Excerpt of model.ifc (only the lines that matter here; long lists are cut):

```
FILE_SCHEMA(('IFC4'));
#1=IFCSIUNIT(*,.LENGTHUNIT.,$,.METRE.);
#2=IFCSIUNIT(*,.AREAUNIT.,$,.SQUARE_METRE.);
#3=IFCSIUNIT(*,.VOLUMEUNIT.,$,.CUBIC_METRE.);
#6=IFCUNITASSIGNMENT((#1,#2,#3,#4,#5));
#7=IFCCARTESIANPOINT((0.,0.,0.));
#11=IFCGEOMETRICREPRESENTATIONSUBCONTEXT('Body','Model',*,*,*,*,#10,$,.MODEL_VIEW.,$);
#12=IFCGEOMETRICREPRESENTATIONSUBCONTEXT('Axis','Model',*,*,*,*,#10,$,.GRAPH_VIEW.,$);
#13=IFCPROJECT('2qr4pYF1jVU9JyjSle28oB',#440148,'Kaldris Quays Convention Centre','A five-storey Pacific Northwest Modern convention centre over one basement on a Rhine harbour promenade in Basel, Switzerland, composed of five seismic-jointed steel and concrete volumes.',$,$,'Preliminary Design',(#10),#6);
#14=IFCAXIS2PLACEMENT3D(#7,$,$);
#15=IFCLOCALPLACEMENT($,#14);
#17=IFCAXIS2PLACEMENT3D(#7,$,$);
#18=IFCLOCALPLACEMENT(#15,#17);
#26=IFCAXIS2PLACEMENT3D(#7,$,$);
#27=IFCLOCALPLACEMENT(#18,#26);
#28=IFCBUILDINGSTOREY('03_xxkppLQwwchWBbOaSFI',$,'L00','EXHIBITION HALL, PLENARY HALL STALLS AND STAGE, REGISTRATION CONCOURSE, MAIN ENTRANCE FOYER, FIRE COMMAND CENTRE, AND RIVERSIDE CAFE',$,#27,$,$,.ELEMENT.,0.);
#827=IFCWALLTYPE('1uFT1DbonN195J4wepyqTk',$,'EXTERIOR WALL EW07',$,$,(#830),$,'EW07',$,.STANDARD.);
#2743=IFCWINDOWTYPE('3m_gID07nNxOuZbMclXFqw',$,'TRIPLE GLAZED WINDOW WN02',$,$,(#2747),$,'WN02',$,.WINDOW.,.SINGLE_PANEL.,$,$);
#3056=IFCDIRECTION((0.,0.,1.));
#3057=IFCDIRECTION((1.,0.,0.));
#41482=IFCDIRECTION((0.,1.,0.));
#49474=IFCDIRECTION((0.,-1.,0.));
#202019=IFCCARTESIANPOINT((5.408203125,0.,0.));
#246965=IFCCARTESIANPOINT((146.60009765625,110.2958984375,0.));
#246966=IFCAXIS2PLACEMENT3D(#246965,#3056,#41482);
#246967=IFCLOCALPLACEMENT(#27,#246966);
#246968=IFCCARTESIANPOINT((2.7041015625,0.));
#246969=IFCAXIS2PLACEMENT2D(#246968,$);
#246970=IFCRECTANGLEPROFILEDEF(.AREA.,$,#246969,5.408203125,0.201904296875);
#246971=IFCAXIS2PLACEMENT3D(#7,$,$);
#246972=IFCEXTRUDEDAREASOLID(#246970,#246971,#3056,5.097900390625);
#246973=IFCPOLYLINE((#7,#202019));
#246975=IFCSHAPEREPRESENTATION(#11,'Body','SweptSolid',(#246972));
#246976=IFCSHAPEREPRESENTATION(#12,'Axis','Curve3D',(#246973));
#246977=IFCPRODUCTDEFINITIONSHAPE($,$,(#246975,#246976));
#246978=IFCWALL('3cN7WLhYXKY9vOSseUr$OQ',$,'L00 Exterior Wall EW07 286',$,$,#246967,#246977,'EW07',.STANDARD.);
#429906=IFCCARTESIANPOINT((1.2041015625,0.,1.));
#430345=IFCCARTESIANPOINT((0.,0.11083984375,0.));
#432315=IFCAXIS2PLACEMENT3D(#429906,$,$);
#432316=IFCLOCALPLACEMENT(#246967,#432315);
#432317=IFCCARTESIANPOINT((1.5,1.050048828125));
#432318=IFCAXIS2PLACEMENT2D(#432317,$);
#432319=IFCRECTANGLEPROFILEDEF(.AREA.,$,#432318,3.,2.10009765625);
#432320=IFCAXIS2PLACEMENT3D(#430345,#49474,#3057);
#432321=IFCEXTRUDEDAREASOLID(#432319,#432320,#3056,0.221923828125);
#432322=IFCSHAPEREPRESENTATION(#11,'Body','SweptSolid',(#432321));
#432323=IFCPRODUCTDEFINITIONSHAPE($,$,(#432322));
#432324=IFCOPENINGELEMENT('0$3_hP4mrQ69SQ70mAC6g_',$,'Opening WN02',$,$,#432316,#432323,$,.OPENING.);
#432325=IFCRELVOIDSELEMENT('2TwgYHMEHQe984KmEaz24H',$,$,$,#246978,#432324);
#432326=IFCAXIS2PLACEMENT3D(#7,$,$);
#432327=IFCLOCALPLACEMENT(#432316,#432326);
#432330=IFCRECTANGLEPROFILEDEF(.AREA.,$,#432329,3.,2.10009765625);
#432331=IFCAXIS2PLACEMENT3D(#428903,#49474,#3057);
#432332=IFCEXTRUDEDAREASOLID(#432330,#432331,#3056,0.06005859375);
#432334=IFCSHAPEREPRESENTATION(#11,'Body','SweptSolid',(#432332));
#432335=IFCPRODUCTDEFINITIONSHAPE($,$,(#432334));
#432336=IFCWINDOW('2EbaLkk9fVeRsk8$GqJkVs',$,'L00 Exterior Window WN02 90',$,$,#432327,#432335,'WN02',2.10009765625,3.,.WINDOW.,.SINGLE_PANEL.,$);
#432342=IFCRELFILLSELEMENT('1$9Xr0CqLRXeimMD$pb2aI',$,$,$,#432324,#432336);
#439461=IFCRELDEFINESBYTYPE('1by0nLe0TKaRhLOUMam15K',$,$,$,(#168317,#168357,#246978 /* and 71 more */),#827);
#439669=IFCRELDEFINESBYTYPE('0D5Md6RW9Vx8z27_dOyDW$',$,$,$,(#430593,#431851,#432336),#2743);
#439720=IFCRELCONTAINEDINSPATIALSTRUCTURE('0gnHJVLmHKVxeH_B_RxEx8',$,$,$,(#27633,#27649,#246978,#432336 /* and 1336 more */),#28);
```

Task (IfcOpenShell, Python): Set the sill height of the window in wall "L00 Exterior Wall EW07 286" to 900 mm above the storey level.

```python
import numpy as np
import ifcopenshell
import ifcopenshell.api.geometry
import ifcopenshell.geom
import ifcopenshell.util.element
import ifcopenshell.util.placement
import ifcopenshell.util.shape
import ifcopenshell.util.unit

model = ifcopenshell.open("model.ifc")
unit_scale = ifcopenshell.util.unit.calculate_unit_scale(model)

window = model.by_id(432336)
opening = window.FillsVoids[0].RelatingOpeningElement
storey = ifcopenshell.util.element.get_container(window, ifc_class="IfcBuildingStorey")
level = ifcopenshell.util.placement.get_local_placement(storey.ObjectPlacement)[2, 3]

# The opening's origin need not be at the sill, so measure its lowest point.
shape = ifcopenshell.geom.create_shape(ifcopenshell.geom.settings(), opening)
bottom = ifcopenshell.util.shape.get_shape_bottom_elevation(shape, shape.geometry) / unit_scale
dz = level + 0.9 / unit_scale - bottom

shift = np.array([0.0, 0.0, dz])
# The window is placed relative to its opening, so it follows when the opening moves.
matrix = ifcopenshell.util.placement.get_local_placement(opening.ObjectPlacement)
matrix[:3, 3] += shift
ifcopenshell.api.geometry.edit_object_placement(
    model, product=opening, matrix=matrix, is_si=False, should_transform_children=True
)

print(f"moved by {dz * unit_scale:+.3f} m")

model.write("model_v2.ifc")
```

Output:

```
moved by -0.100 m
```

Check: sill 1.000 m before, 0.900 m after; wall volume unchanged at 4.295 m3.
